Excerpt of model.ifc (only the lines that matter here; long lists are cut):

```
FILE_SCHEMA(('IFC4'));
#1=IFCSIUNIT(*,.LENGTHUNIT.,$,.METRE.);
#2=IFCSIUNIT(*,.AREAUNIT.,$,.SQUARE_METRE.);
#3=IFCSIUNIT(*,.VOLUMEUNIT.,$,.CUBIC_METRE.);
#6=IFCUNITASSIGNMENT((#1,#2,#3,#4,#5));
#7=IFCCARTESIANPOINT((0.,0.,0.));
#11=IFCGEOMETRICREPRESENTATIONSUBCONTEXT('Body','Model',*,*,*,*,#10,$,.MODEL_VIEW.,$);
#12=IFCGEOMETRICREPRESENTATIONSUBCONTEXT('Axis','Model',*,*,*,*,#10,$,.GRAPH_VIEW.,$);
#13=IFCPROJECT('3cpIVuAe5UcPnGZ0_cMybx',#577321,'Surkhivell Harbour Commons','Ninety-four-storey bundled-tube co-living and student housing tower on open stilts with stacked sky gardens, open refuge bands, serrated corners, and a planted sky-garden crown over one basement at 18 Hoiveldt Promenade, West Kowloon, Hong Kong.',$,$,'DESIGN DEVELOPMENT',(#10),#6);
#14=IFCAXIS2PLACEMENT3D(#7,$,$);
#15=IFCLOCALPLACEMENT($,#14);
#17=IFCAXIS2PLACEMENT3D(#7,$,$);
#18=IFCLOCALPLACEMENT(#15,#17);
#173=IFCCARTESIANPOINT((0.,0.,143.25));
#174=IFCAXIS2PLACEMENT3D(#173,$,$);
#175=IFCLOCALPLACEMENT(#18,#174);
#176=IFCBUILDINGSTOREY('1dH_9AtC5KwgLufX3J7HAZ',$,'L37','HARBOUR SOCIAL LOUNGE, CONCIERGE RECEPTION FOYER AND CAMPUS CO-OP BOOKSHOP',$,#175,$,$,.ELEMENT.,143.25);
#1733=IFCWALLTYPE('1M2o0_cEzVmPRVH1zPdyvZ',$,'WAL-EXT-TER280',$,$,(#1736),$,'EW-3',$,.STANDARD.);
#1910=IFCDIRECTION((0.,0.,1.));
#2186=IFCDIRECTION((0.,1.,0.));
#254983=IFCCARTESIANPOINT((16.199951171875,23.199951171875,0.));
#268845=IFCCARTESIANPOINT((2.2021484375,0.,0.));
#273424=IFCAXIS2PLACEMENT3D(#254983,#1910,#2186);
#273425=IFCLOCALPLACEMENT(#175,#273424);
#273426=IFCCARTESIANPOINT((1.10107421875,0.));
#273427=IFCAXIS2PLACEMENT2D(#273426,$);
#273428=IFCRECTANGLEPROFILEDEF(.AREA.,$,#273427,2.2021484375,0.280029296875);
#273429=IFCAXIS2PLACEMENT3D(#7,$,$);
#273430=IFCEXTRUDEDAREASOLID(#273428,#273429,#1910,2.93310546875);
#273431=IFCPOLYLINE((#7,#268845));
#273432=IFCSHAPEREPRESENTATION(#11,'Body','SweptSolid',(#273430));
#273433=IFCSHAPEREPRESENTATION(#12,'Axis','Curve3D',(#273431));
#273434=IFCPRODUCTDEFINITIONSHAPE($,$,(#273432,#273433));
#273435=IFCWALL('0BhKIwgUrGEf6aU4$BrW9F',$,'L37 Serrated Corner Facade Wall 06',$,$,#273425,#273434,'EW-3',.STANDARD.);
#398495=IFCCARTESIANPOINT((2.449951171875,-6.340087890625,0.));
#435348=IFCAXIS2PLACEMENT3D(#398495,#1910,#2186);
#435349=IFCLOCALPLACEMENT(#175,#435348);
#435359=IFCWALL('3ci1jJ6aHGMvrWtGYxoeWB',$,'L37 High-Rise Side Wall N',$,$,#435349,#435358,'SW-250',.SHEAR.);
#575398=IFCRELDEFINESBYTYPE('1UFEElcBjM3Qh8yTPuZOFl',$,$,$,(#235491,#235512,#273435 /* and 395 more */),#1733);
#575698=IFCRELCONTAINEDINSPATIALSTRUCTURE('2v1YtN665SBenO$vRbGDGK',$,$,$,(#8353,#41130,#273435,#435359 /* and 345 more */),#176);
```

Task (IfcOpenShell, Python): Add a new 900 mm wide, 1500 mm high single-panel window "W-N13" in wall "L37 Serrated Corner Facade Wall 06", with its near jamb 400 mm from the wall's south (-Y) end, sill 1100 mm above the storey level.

```python
import numpy as np
import ifcopenshell
import ifcopenshell.api.feature
import ifcopenshell.api.geometry
import ifcopenshell.api.root
import ifcopenshell.api.spatial
import ifcopenshell.geom
import ifcopenshell.util.element
import ifcopenshell.util.placement
import ifcopenshell.util.representation
import ifcopenshell.util.shape
import ifcopenshell.util.unit

model = ifcopenshell.open("model.ifc")
unit_scale = ifcopenshell.util.unit.calculate_unit_scale(model)
settings = ifcopenshell.geom.settings()


def volume(element):
    """Net volume in cubic metres, openings subtracted."""
    shape = ifcopenshell.geom.create_shape(settings, element)
    return ifcopenshell.util.shape.get_volume(shape.geometry)


wall = model.by_guid("0BhKIwgUrGEf6aU4$BrW9F")
storey = ifcopenshell.util.element.get_container(wall, ifc_class="IfcBuildingStorey")
context = ifcopenshell.util.representation.get_context(model, "Model", "Body", "MODEL_VIEW")
before = volume(wall)

width, height, from_end, sill = 0.9, 1.5, 0.4, 1.1  # metres

# The wall runs along its own X axis, and the end named is its -X end.
wall_shape = ifcopenshell.geom.create_shape(settings, wall)
x, y, z = ifcopenshell.util.shape.get_vertices(wall_shape.geometry).T
start = x.min() + from_end
face, thickness = float(y.min()), float(y.max() - y.min())
wall_matrix = ifcopenshell.util.placement.get_local_placement(wall.ObjectPlacement)
level = ifcopenshell.util.placement.get_local_placement(storey.ObjectPlacement)[2, 3]


def in_wall(x, y):
    """Placement at x, y metres in the wall's axes, at sill height."""
    matrix = wall_matrix.copy()
    matrix[:, 3] = wall_matrix @ np.array([x / unit_scale, y / unit_scale, 0.0, 1.0])
    matrix[2, 3] = level + sill / unit_scale
    return matrix


# Opening: a box that overshoots both wall faces by 50 mm.
opening = ifcopenshell.api.root.create_entity(model, ifc_class="IfcOpeningElement", predefined_type="OPENING")
box = ifcopenshell.api.geometry.add_wall_representation(
    model, context=context, length=width, height=height, thickness=thickness + 0.1
)
ifcopenshell.api.geometry.assign_representation(model, product=opening, representation=box)
ifcopenshell.api.geometry.edit_object_placement(model, product=opening, matrix=in_wall(start, face - 0.05), is_si=False)
ifcopenshell.api.feature.add_feature(model, feature=opening, element=wall)

window = ifcopenshell.api.root.create_entity(model, ifc_class="IfcWindow", name="W-N13", predefined_type="WINDOW")
window.OverallWidth, window.OverallHeight = width / unit_scale, height / unit_scale
window.PartitioningType = "SINGLE_PANEL"
body = ifcopenshell.api.geometry.add_window_representation(
    model,
    context=context,
    overall_width=window.OverallWidth,
    overall_height=window.OverallHeight,
    partition_type="SINGLE_PANEL",
)
ifcopenshell.api.geometry.assign_representation(model, product=window, representation=body)
ifcopenshell.api.spatial.assign_container(model, products=[window], relating_structure=storey)
ifcopenshell.api.feature.add_filling(model, opening=opening, element=window)

# Centre the window in the wall's thickness.
ifcopenshell.api.geometry.edit_object_placement(model, product=window, matrix=in_wall(start, face), is_si=False)
window_shape = ifcopenshell.geom.create_shape(settings, window)
depth = ifcopenshell.util.shape.get_vertices(window_shape.geometry)[:, 1]
offset = face + thickness / 2 - (depth.min() + depth.max()) / 2
ifcopenshell.api.geometry.edit_object_placement(model, product=window, matrix=in_wall(start, offset), is_si=False)

after = volume(wall)

print(f"wall volume {before:.3f} -> {after:.3f} m3")

model.write("model_edited.ifc")
```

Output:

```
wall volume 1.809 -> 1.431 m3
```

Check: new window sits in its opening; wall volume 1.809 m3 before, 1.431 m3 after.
